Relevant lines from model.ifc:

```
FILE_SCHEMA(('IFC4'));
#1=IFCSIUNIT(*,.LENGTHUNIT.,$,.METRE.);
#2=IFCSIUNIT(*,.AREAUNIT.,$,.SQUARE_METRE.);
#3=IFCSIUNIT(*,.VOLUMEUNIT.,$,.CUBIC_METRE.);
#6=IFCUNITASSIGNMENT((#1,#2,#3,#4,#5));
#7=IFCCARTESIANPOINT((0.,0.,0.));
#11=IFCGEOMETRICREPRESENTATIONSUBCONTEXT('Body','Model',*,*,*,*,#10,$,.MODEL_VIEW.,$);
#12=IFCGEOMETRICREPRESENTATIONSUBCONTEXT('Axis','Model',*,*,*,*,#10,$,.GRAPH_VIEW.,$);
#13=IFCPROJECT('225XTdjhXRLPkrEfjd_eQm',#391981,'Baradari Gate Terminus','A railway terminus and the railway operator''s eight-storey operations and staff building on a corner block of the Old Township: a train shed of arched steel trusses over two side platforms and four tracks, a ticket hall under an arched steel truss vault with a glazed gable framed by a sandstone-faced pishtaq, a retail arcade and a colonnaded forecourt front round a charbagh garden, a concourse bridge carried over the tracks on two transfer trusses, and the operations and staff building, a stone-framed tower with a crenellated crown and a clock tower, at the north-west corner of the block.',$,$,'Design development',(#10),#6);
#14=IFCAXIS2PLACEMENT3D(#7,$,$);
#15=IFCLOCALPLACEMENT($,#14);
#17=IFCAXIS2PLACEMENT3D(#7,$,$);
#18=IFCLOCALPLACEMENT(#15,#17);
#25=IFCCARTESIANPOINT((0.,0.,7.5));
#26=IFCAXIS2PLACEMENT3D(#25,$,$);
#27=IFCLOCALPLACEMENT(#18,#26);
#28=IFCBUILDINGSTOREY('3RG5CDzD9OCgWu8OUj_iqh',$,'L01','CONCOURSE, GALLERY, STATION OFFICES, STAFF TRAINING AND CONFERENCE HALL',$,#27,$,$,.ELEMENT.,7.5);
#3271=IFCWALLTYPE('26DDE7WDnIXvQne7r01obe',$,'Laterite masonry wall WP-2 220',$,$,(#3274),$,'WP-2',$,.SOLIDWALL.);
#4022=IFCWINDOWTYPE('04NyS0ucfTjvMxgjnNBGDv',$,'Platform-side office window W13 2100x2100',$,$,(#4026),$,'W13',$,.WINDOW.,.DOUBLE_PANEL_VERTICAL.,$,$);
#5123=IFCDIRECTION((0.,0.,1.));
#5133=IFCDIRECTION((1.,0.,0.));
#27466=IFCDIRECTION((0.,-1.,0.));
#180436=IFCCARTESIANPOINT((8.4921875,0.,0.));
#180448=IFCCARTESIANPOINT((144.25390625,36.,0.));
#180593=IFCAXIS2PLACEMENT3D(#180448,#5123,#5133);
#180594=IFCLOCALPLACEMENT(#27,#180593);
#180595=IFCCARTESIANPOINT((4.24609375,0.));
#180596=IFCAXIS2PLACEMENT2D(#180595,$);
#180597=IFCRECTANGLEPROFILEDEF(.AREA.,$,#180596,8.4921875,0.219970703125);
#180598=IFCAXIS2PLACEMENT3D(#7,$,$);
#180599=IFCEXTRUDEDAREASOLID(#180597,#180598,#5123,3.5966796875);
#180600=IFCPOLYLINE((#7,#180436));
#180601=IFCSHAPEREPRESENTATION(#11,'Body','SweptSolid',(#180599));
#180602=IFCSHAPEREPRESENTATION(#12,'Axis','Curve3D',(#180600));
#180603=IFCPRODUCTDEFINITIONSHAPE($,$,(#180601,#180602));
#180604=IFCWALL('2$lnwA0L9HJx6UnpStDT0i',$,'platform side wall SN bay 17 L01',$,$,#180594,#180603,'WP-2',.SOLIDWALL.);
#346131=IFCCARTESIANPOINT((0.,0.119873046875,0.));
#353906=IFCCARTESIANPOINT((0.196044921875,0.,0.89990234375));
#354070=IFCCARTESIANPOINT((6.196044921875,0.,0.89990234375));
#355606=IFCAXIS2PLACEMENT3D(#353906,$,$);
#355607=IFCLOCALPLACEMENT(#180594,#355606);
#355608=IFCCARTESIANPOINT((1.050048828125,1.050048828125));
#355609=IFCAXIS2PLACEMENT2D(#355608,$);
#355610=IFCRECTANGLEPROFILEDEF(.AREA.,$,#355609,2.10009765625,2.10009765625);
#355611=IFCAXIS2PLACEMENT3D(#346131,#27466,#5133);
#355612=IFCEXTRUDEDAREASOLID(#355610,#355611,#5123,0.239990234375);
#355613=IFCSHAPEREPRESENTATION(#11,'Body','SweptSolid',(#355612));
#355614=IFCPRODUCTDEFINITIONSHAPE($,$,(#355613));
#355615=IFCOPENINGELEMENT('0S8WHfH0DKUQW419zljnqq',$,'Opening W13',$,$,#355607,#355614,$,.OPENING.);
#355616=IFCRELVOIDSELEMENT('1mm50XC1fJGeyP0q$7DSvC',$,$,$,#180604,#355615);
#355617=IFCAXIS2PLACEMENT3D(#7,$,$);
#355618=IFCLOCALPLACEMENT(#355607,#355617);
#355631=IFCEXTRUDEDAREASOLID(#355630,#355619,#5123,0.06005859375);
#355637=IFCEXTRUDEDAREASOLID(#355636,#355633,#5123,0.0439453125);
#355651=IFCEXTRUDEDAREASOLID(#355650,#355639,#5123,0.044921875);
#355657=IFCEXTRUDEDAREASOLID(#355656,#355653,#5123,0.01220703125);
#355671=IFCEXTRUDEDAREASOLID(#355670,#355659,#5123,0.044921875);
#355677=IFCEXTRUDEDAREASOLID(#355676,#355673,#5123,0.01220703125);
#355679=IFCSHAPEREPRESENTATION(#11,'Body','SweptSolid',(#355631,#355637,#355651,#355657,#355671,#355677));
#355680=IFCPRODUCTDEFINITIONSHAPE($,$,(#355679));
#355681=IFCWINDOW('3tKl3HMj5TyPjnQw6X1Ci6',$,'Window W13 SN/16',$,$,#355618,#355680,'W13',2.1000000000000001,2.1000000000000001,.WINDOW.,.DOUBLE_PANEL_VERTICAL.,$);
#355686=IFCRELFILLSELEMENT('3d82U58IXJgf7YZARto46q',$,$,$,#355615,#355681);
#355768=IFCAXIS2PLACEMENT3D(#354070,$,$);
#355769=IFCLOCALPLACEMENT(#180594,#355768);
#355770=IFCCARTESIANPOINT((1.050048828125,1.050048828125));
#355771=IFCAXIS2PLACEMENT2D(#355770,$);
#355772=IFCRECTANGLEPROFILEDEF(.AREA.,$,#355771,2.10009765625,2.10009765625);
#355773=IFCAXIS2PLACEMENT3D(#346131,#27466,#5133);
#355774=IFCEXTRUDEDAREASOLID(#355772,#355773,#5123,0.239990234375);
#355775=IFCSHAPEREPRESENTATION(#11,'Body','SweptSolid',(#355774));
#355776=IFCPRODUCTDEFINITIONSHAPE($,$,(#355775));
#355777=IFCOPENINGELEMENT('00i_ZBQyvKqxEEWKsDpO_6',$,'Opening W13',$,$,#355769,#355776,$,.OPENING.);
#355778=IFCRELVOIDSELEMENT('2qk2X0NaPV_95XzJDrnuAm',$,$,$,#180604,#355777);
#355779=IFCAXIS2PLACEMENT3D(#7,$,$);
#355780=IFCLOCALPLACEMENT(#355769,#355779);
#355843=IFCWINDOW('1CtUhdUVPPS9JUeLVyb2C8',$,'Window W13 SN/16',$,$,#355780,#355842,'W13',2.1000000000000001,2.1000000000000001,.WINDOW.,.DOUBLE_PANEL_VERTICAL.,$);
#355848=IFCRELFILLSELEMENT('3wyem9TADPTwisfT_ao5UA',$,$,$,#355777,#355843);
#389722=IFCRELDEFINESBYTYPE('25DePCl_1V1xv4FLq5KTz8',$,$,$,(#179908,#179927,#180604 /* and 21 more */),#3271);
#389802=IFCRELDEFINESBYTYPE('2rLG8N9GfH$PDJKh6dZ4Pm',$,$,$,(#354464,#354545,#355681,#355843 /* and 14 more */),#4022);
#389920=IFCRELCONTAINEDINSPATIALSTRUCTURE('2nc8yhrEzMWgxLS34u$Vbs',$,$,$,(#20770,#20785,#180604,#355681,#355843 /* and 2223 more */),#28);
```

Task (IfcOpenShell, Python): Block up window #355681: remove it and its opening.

```python
import ifcopenshell
import ifcopenshell.api.feature
import ifcopenshell.api.root
import ifcopenshell.geom
import ifcopenshell.util.shape

model = ifcopenshell.open("model.ifc")
settings = ifcopenshell.geom.settings()


def volume(element):
    """Net volume in cubic metres, openings subtracted."""
    shape = ifcopenshell.geom.create_shape(settings, element)
    return ifcopenshell.util.shape.get_volume(shape.geometry)


window = model.by_guid("3tKl3HMj5TyPjnQw6X1Ci6")
opening = window.FillsVoids[0].RelatingOpeningElement
wall = opening.VoidsElements[0].RelatingBuildingElement
before = volume(wall)

ifcopenshell.api.root.remove_product(model, product=window)
ifcopenshell.api.feature.remove_feature(model, feature=opening)

after = volume(wall)

print(f"wall volume {before:.3f} -> {after:.3f} m3")

model.write("model_v2.ifc")
```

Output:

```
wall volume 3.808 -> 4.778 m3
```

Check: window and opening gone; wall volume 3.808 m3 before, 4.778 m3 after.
